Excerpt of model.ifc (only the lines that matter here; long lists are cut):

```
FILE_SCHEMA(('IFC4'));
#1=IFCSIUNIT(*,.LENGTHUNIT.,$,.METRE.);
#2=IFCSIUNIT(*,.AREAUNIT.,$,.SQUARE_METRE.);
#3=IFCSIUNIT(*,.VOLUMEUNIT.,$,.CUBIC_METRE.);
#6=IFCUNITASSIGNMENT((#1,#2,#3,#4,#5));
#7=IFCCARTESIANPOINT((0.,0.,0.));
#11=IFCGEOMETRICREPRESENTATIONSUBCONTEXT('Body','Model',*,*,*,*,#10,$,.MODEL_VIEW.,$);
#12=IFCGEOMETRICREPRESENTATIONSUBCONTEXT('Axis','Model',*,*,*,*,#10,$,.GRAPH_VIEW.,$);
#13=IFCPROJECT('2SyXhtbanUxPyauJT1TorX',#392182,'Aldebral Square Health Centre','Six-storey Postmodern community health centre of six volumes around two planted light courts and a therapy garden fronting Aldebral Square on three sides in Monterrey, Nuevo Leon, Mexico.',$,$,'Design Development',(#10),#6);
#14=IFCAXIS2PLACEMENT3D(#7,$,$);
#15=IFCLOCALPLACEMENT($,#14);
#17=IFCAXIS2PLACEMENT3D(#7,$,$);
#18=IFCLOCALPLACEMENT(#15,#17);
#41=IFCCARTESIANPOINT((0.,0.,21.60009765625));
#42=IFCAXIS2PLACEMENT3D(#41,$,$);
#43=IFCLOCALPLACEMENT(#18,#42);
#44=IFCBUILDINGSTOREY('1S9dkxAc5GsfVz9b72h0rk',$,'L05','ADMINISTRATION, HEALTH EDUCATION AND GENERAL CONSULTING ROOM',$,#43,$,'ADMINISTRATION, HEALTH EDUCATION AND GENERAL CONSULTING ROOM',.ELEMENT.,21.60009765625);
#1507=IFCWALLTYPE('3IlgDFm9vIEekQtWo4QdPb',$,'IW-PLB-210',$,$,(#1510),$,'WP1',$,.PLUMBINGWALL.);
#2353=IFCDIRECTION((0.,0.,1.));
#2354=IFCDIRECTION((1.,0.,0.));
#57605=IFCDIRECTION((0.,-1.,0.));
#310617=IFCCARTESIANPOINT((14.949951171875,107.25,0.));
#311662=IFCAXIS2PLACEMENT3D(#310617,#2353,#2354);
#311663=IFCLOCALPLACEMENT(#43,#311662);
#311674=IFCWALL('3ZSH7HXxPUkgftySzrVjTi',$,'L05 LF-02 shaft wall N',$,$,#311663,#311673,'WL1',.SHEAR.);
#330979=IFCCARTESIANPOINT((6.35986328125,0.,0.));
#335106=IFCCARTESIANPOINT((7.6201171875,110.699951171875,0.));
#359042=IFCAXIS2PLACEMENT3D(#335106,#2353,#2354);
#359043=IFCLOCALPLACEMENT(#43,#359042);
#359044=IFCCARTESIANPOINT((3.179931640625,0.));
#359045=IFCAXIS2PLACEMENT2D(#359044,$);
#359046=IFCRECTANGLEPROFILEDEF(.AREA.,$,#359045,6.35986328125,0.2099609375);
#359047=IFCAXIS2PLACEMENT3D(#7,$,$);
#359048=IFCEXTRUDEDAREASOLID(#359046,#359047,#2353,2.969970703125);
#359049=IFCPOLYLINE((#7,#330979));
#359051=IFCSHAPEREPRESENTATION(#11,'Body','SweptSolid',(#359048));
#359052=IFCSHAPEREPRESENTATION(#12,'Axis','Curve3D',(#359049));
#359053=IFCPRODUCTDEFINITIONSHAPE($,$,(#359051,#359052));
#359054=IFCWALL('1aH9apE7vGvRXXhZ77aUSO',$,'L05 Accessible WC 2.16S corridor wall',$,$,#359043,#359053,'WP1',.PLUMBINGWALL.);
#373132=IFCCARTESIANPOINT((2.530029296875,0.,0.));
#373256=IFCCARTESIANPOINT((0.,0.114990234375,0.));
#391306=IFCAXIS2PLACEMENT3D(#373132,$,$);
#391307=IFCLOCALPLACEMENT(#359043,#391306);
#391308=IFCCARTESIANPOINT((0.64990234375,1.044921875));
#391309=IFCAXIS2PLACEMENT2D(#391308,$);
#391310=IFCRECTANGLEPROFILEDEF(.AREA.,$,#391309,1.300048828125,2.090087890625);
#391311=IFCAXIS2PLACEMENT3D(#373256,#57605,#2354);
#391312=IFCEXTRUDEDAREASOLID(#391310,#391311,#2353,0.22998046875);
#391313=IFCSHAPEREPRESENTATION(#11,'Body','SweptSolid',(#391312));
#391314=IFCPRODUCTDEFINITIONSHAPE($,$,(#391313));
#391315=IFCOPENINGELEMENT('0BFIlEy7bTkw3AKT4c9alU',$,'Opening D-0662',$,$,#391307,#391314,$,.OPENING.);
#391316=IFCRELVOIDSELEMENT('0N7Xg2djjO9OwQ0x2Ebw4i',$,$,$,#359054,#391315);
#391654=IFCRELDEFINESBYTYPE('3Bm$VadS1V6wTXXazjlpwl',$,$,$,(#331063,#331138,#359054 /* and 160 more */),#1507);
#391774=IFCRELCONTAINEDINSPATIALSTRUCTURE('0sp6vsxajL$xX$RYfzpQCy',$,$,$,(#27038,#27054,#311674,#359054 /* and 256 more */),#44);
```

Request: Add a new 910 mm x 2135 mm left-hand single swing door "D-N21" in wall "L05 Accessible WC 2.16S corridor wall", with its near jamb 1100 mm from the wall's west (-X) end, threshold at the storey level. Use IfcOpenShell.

```python
import numpy as np
import ifcopenshell
import ifcopenshell.api.feature
import ifcopenshell.api.geometry
import ifcopenshell.api.root
import ifcopenshell.api.spatial
import ifcopenshell.geom
import ifcopenshell.util.element
import ifcopenshell.util.placement
import ifcopenshell.util.representation
import ifcopenshell.util.shape
import ifcopenshell.util.unit

model = ifcopenshell.open("model.ifc")
unit_scale = ifcopenshell.util.unit.calculate_unit_scale(model)
settings = ifcopenshell.geom.settings()


def volume(element):
    """Net volume in cubic metres, openings subtracted."""
    shape = ifcopenshell.geom.create_shape(settings, element)
    return ifcopenshell.util.shape.get_volume(shape.geometry)


wall = model.by_guid("1aH9apE7vGvRXXhZ77aUSO")
storey = ifcopenshell.util.element.get_container(wall, ifc_class="IfcBuildingStorey")
context = ifcopenshell.util.representation.get_context(model, "Model", "Body", "MODEL_VIEW")
before = volume(wall)

width, height, from_end, sill = 0.91, 2.135, 1.1, 0.0  # metres

# The wall runs along its own X axis, and the end named is its -X end.
wall_shape = ifcopenshell.geom.create_shape(settings, wall)
x, y, z = ifcopenshell.util.shape.get_vertices(wall_shape.geometry).T
start = x.min() + from_end
face, thickness = float(y.min()), float(y.max() - y.min())
wall_matrix = ifcopenshell.util.placement.get_local_placement(wall.ObjectPlacement)
level = ifcopenshell.util.placement.get_local_placement(storey.ObjectPlacement)[2, 3]


def in_wall(x, y):
    """Placement at x, y metres in the wall's axes, at sill height."""
    matrix = wall_matrix.copy()
    matrix[:, 3] = wall_matrix @ np.array([x / unit_scale, y / unit_scale, 0.0, 1.0])
    matrix[2, 3] = level + sill / unit_scale
    return matrix


# Opening: a box that overshoots both wall faces by 50 mm.
opening = ifcopenshell.api.root.create_entity(model, ifc_class="IfcOpeningElement", predefined_type="OPENING")
box = ifcopenshell.api.geometry.add_wall_representation(
    model, context=context, length=width, height=height, thickness=thickness + 0.1
)
ifcopenshell.api.geometry.assign_representation(model, product=opening, representation=box)
ifcopenshell.api.geometry.edit_object_placement(model, product=opening, matrix=in_wall(start, face - 0.05), is_si=False)
ifcopenshell.api.feature.add_feature(model, feature=opening, element=wall)

door = ifcopenshell.api.root.create_entity(model, ifc_class="IfcDoor", name="D-N21", predefined_type="DOOR")
door.OverallWidth, door.OverallHeight = width / unit_scale, height / unit_scale
door.OperationType = "SINGLE_SWING_LEFT"
body = ifcopenshell.api.geometry.add_door_representation(
    model,
    context=context,
    overall_width=door.OverallWidth,
    overall_height=door.OverallHeight,
    operation_type="SINGLE_SWING_LEFT",
    lining_properties={"LiningDepth": thickness / unit_scale, "ThresholdDepth": thickness / unit_scale},
)
ifcopenshell.api.geometry.assign_representation(model, product=door, representation=body)
ifcopenshell.api.spatial.assign_container(model, products=[door], relating_structure=storey)
ifcopenshell.api.feature.add_filling(model, opening=opening, element=door)

# The lining spans the wall, so the door starts at the wall face.
ifcopenshell.api.geometry.edit_object_placement(model, product=door, matrix=in_wall(start, face), is_si=False)

after = volume(wall)

print(f"wall volume {before:.3f} -> {after:.3f} m3")

model.write("model_edited.ifc")
```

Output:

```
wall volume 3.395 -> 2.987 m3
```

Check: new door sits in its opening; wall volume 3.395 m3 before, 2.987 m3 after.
